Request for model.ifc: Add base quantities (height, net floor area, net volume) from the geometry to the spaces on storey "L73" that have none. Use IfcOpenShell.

First a look at what the model holds.

```python
import ifcopenshell
import ifcopenshell.util.element
import ifcopenshell.util.unit

model = ifcopenshell.open("model.ifc")
print(model.schema)
for unit_type in ("LENGTHUNIT", "AREAUNIT", "VOLUMEUNIT"):
    print(unit_type, ifcopenshell.util.unit.calculate_unit_scale(model, unit_type))
storey = next(s for s in model.by_type("IfcBuildingStorey") if s.Name == "L73")
spaces = [e for e in ifcopenshell.util.element.get_decomposition(storey) if e.is_a("IfcSpace")]
for e in sorted(spaces, key=lambda e: e.id()):
    print(e.id(), e.is_a(), e.Name, list(ifcopenshell.util.element.get_psets(e, qtos_only=True)), sep=" | ")
```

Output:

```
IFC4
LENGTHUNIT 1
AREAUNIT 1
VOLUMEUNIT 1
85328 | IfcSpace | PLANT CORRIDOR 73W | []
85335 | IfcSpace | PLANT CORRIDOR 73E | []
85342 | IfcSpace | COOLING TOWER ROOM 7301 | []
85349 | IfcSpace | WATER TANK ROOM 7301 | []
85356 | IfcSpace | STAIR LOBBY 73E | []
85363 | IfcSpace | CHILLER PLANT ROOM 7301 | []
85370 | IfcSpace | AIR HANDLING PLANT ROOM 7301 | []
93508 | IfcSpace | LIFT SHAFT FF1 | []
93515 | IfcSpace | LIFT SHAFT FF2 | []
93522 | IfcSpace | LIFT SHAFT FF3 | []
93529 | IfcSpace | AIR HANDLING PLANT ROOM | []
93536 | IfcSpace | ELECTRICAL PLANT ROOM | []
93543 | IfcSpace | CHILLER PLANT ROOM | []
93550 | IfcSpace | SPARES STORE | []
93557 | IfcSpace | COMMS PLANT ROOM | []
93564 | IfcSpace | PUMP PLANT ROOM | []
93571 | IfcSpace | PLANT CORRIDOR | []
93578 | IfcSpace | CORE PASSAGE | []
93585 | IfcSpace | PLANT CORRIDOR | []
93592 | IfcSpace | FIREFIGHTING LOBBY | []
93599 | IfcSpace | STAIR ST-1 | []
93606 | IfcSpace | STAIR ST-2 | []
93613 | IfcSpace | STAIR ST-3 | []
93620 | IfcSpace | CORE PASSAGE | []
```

```python
import ifcopenshell
import ifcopenshell.api.pset
import ifcopenshell.geom
import ifcopenshell.util.element
import ifcopenshell.util.shape
import ifcopenshell.util.unit

model = ifcopenshell.open("model.ifc")
unit_scale = ifcopenshell.util.unit.calculate_unit_scale(model)
area_scale = ifcopenshell.util.unit.calculate_unit_scale(model, "AREAUNIT")
volume_scale = ifcopenshell.util.unit.calculate_unit_scale(model, "VOLUMEUNIT")
settings = ifcopenshell.geom.settings()

storey = next(s for s in model.by_type("IfcBuildingStorey") if s.Name == "L73")
spaces = [e for e in ifcopenshell.util.element.get_decomposition(storey) if e.is_a("IfcSpace")]

for e in sorted(spaces, key=lambda e: e.id()):
    if ifcopenshell.util.element.get_psets(e, qtos_only=True, should_inherit=False):
        continue
    # Geometry comes back in metres, in the element's own axes.
    shape = ifcopenshell.geom.create_shape(settings, e)
    values = {
        "Height": ifcopenshell.util.shape.get_z(shape.geometry) / unit_scale,
        "NetFloorArea": ifcopenshell.util.shape.get_footprint_area(shape.geometry) / area_scale,
        "NetVolume": ifcopenshell.util.shape.get_volume(shape.geometry) / volume_scale,
    }
    qto = ifcopenshell.api.pset.add_qto(model, product=e, name="Qto_SpaceBaseQuantities")
    ifcopenshell.api.pset.edit_qto(model, qto=qto, properties=values)
    print(e.id(), {k: round(v, 3) for k, v in values.items()})

model.write("model_rev.ifc")
```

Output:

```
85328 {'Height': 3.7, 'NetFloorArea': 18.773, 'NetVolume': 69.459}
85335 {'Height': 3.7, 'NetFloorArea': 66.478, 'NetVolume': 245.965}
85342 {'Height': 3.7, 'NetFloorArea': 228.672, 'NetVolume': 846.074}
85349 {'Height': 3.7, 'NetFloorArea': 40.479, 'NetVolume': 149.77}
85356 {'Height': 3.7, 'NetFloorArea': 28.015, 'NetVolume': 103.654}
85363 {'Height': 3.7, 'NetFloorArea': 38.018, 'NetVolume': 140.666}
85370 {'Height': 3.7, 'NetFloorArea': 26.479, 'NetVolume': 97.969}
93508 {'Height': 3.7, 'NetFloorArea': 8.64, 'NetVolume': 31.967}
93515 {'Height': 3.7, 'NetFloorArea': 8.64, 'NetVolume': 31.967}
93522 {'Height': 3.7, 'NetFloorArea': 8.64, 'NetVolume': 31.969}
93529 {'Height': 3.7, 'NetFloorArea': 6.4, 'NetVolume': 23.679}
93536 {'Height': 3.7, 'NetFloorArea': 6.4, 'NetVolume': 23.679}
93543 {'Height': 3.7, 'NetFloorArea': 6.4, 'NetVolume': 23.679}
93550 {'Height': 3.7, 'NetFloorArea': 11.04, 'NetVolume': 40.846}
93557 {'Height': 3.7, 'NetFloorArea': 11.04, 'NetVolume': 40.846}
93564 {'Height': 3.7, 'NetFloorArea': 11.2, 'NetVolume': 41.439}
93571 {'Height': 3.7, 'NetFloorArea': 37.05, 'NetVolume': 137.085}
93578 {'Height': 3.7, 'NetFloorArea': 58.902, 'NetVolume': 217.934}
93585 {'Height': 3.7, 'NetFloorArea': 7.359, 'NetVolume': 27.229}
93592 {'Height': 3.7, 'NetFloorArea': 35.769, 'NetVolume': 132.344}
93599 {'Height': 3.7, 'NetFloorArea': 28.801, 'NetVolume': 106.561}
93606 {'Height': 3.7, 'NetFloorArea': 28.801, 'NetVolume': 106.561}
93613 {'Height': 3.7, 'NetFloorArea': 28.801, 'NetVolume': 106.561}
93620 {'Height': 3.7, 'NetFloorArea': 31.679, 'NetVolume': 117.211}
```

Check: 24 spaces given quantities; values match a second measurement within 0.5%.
